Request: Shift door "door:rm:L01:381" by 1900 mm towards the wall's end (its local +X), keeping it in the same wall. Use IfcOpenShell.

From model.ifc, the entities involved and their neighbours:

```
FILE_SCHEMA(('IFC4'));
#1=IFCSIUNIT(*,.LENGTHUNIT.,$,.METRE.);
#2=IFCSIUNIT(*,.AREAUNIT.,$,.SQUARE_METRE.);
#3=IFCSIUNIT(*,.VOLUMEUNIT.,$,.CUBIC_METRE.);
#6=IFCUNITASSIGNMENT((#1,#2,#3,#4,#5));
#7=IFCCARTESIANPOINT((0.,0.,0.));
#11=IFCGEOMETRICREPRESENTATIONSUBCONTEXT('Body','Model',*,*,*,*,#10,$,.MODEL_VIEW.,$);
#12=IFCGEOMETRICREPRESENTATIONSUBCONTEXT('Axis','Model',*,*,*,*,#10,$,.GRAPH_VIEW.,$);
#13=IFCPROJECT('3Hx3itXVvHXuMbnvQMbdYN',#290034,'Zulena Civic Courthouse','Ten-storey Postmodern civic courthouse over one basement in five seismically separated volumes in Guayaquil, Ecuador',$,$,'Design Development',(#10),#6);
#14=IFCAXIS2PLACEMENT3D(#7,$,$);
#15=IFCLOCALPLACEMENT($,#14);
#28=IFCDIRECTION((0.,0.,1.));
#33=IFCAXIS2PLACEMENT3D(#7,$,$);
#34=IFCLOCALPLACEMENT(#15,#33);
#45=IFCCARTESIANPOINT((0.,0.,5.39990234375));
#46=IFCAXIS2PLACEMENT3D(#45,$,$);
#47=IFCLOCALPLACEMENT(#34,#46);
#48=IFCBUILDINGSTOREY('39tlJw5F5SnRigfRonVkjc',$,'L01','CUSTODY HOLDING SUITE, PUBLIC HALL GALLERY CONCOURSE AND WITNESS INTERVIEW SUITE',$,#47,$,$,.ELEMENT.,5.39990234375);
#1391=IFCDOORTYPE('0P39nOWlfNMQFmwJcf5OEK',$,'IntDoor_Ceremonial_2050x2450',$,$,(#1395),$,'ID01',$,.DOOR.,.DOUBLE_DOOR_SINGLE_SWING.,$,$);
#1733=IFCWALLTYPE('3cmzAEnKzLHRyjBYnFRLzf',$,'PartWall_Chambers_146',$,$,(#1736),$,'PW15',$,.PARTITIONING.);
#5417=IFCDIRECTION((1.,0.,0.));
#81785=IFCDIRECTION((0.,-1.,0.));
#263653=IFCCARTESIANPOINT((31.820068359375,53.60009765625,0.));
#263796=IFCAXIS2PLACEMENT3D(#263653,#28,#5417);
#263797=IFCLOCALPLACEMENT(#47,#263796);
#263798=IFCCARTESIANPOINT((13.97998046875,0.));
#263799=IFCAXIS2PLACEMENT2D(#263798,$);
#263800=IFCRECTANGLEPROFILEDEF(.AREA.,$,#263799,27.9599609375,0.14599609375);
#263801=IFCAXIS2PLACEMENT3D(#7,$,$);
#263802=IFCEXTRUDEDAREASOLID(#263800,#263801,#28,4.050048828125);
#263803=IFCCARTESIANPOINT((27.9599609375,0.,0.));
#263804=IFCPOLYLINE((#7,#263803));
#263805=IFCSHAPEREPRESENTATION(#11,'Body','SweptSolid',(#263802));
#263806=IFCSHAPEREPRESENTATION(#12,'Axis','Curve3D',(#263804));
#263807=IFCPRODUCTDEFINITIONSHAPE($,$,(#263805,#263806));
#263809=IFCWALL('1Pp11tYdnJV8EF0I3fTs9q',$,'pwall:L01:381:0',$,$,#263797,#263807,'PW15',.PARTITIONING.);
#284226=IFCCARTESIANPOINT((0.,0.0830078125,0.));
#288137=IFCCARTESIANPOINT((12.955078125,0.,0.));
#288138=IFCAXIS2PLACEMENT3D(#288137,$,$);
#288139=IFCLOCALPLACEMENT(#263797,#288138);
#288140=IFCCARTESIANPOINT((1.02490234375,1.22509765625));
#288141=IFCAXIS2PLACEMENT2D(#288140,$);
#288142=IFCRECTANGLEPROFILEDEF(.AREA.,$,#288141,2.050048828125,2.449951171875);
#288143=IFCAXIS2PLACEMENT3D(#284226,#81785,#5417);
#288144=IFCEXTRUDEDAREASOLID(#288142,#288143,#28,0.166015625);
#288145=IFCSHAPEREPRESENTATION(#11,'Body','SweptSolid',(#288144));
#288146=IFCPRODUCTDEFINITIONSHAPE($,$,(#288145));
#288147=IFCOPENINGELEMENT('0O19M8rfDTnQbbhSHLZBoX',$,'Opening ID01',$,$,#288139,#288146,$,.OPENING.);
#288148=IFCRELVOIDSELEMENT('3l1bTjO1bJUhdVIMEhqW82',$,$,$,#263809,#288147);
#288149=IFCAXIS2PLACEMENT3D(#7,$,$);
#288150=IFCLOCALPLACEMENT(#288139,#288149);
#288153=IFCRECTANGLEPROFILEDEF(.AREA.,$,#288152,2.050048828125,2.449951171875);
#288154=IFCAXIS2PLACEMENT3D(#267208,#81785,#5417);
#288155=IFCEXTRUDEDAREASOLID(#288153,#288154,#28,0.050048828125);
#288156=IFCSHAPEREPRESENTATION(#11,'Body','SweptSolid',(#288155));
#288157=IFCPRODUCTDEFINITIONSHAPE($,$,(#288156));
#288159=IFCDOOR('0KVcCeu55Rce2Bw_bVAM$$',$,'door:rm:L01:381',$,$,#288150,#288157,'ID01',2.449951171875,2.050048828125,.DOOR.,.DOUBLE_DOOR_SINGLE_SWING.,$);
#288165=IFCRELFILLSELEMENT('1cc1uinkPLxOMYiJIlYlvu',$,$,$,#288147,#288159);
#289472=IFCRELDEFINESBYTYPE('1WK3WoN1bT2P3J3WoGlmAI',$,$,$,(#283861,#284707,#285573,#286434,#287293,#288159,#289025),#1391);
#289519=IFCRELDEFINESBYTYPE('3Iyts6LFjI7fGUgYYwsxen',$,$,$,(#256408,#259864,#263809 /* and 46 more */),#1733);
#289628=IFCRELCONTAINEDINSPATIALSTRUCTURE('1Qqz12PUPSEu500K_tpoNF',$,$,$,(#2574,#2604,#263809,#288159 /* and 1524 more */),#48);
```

```python
import ifcopenshell
import ifcopenshell.api.geometry
import ifcopenshell.util.placement
import ifcopenshell.util.unit

model = ifcopenshell.open("model.ifc")
unit_scale = ifcopenshell.util.unit.calculate_unit_scale(model)

door = model.by_guid("0KVcCeu55Rce2Bw_bVAM$$")
opening = door.FillsVoids[0].RelatingOpeningElement
wall = opening.VoidsElements[0].RelatingBuildingElement

wall_matrix = ifcopenshell.util.placement.get_local_placement(wall.ObjectPlacement)
shift = wall_matrix[:3, 0] * 1.9 / unit_scale
before = ifcopenshell.util.placement.get_local_placement(door.ObjectPlacement)[:3, 3].copy()

# The door is placed relative to its opening, so it follows when the opening moves.
matrix = ifcopenshell.util.placement.get_local_placement(opening.ObjectPlacement)
matrix[:3, 3] += shift
ifcopenshell.api.geometry.edit_object_placement(
    model, product=opening, matrix=matrix, is_si=False, should_transform_children=True
)

after = ifcopenshell.util.placement.get_local_placement(door.ObjectPlacement)[:3, 3]
print("door moved by", (after - before).round(3) + 0.0)

model.write("model_v2.ifc")
```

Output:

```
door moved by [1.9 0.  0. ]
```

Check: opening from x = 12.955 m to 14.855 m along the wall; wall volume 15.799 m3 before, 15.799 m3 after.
